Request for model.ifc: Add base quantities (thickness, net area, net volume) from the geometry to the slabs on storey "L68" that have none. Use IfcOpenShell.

First a look at what the model holds.

```python
import ifcopenshell
import ifcopenshell.util.element
import ifcopenshell.util.unit

model = ifcopenshell.open("model.ifc")
print(model.schema)
for unit_type in ("LENGTHUNIT", "AREAUNIT", "VOLUMEUNIT"):
    print(unit_type, ifcopenshell.util.unit.calculate_unit_scale(model, unit_type))
storey = next(s for s in model.by_type("IfcBuildingStorey") if s.Name == "L68")
slabs = [e for e in ifcopenshell.util.element.get_decomposition(storey) if e.is_a("IfcSlab")]
for e in sorted(slabs, key=lambda e: e.id()):
    print(e.id(), e.is_a(), e.Name, list(ifcopenshell.util.element.get_psets(e, qtos_only=True)), sep=" | ")
```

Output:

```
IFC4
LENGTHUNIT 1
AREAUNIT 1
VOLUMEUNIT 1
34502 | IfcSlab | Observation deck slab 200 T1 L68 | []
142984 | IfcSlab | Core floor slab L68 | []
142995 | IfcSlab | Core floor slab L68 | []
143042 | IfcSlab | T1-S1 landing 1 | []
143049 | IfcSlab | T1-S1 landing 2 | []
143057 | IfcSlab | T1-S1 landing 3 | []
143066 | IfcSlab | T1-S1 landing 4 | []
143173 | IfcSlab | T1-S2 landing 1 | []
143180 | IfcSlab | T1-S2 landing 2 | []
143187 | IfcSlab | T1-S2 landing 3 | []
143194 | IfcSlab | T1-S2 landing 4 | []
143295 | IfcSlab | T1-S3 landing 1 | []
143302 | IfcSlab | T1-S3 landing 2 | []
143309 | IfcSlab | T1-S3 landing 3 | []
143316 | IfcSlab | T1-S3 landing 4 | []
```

```python
import ifcopenshell
import ifcopenshell.api.pset
import ifcopenshell.geom
import ifcopenshell.util.element
import ifcopenshell.util.shape
import ifcopenshell.util.unit

model = ifcopenshell.open("model.ifc")
unit_scale = ifcopenshell.util.unit.calculate_unit_scale(model)
area_scale = ifcopenshell.util.unit.calculate_unit_scale(model, "AREAUNIT")
volume_scale = ifcopenshell.util.unit.calculate_unit_scale(model, "VOLUMEUNIT")
settings = ifcopenshell.geom.settings()

storey = next(s for s in model.by_type("IfcBuildingStorey") if s.Name == "L68")
slabs = [e for e in ifcopenshell.util.element.get_decomposition(storey) if e.is_a("IfcSlab")]

for e in sorted(slabs, key=lambda e: e.id()):
    if ifcopenshell.util.element.get_psets(e, qtos_only=True, should_inherit=False):
        continue
    # Geometry comes back in metres, in the element's own axes.
    shape = ifcopenshell.geom.create_shape(settings, e)
    values = {
        "Width": ifcopenshell.util.shape.get_z(shape.geometry) / unit_scale,
        "NetArea": ifcopenshell.util.shape.get_footprint_area(shape.geometry) / area_scale,
        "NetVolume": ifcopenshell.util.shape.get_volume(shape.geometry) / volume_scale,
    }
    qto = ifcopenshell.api.pset.add_qto(model, product=e, name="Qto_SlabBaseQuantities")
    ifcopenshell.api.pset.edit_qto(model, qto=qto, properties=values)
    print(e.id(), {k: round(v, 3) for k, v in values.items()})

model.write("model_v2.ifc")
```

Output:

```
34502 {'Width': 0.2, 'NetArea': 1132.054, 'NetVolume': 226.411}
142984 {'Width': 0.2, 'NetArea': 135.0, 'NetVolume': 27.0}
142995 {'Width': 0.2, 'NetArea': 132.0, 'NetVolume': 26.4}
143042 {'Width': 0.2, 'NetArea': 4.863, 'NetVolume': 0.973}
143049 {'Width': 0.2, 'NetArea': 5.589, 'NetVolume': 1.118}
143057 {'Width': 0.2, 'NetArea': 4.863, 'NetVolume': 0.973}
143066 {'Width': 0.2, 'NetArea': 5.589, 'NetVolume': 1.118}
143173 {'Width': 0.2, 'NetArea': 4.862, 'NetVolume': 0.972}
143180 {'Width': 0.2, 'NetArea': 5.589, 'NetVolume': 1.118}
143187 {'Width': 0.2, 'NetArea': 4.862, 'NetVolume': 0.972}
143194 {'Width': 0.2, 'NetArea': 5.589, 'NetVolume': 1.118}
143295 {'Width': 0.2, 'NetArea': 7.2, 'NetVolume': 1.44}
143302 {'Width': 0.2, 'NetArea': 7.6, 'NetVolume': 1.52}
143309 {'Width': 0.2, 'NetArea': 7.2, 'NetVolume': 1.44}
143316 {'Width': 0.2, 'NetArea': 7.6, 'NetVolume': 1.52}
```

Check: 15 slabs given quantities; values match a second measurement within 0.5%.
